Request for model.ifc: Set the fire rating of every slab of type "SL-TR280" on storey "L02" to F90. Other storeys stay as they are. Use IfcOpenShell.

First a look at what the model holds.

```python
import ifcopenshell
import ifcopenshell.util.element

model = ifcopenshell.open("model.ifc")
print(model.schema)
storey = next(s for s in model.by_type("IfcBuildingStorey") if s.Name == "L02")
slabs = [e for e in ifcopenshell.util.element.get_decomposition(storey) if e.is_a("IfcSlab")]
seen = {}
for e in slabs:
    element_type = ifcopenshell.util.element.get_type(e)
    key = (element_type.Name if element_type != e and element_type else None, ifcopenshell.util.element.get_pset(e, "Pset_SlabCommon", "FireRating"))
    seen[key] = seen.get(key, 0) + 1
for (name, value), count in sorted(seen.items(), key=str):
    print(count, "x", name, "|", value)
```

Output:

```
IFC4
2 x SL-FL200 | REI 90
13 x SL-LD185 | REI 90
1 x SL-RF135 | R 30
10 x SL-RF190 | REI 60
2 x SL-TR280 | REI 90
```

```python
import ifcopenshell
import ifcopenshell.api.pset
import ifcopenshell.util.element

model = ifcopenshell.open("model.ifc")

storey = next(s for s in model.by_type("IfcBuildingStorey") if s.Name == "L02")
slabs = [e for e in ifcopenshell.util.element.get_decomposition(storey) if e.is_a("IfcSlab")]

count = 0
for e in slabs:
    element_type = ifcopenshell.util.element.get_type(e)
    if element_type in (None, e) or element_type.Name != "SL-TR280":
        continue
    # add_pset returns the element's existing set when there is one.
    pset = ifcopenshell.api.pset.add_pset(model, product=e, name="Pset_SlabCommon")
    ifcopenshell.api.pset.edit_pset(model, pset=pset, properties={"FireRating": "F90"})
    count += 1

print(count, "slabs updated")

model.write("model_updated.ifc")
```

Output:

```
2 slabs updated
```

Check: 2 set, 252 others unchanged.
